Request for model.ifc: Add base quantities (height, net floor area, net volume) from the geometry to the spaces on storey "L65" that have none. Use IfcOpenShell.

First a look at what the model holds.

```python
import ifcopenshell
import ifcopenshell.util.element
import ifcopenshell.util.unit

model = ifcopenshell.open("model.ifc")
print(model.schema)
for unit_type in ("LENGTHUNIT", "AREAUNIT", "VOLUMEUNIT"):
    print(unit_type, ifcopenshell.util.unit.calculate_unit_scale(model, unit_type))
storey = next(s for s in model.by_type("IfcBuildingStorey") if s.Name == "L65")
spaces = [e for e in ifcopenshell.util.element.get_decomposition(storey) if e.is_a("IfcSpace")]
for e in sorted(spaces, key=lambda e: e.id()):
    print(e.id(), e.is_a(), e.Name, list(ifcopenshell.util.element.get_psets(e, qtos_only=True)), sep=" | ")
```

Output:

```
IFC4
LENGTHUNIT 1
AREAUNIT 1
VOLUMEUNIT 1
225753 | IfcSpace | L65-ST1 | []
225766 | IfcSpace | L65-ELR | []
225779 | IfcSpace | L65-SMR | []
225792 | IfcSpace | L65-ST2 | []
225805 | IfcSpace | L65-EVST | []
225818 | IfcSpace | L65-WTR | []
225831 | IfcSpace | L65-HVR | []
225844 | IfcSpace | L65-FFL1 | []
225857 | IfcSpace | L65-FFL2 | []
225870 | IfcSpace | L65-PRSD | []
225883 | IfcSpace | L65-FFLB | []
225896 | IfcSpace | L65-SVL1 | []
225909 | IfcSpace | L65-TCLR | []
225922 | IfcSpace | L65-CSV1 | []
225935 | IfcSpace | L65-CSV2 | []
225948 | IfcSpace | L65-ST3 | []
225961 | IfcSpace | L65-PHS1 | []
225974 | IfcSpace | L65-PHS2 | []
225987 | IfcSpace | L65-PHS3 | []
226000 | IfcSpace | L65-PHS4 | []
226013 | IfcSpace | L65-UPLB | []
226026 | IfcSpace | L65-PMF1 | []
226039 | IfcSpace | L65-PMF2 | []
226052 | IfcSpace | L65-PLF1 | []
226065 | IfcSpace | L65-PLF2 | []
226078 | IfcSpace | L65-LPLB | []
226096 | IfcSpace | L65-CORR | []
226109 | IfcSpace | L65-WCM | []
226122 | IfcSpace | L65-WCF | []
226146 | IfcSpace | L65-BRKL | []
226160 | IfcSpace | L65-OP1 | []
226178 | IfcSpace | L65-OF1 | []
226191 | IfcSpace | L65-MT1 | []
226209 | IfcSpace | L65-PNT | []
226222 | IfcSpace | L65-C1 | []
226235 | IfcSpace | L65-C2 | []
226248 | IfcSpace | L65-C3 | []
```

```python
import ifcopenshell
import ifcopenshell.api.pset
import ifcopenshell.geom
import ifcopenshell.util.element
import ifcopenshell.util.shape
import ifcopenshell.util.unit

model = ifcopenshell.open("model.ifc")
unit_scale = ifcopenshell.util.unit.calculate_unit_scale(model)
area_scale = ifcopenshell.util.unit.calculate_unit_scale(model, "AREAUNIT")
volume_scale = ifcopenshell.util.unit.calculate_unit_scale(model, "VOLUMEUNIT")
settings = ifcopenshell.geom.settings()

storey = next(s for s in model.by_type("IfcBuildingStorey") if s.Name == "L65")
spaces = [e for e in ifcopenshell.util.element.get_decomposition(storey) if e.is_a("IfcSpace")]

for e in sorted(spaces, key=lambda e: e.id()):
    if ifcopenshell.util.element.get_psets(e, qtos_only=True, should_inherit=False):
        continue
    # Geometry comes back in metres, in the element's own axes.
    shape = ifcopenshell.geom.create_shape(settings, e)
    values = {
        "Height": ifcopenshell.util.shape.get_z(shape.geometry) / unit_scale,
        "NetFloorArea": ifcopenshell.util.shape.get_footprint_area(shape.geometry) / area_scale,
        "NetVolume": ifcopenshell.util.shape.get_volume(shape.geometry) / volume_scale,
    }
    qto = ifcopenshell.api.pset.add_qto(model, product=e, name="Qto_SpaceBaseQuantities")
    ifcopenshell.api.pset.edit_qto(model, qto=qto, properties=values)
    print(e.id(), {k: round(v, 3) for k, v in values.items()})

model.write("model_v2.ifc")
```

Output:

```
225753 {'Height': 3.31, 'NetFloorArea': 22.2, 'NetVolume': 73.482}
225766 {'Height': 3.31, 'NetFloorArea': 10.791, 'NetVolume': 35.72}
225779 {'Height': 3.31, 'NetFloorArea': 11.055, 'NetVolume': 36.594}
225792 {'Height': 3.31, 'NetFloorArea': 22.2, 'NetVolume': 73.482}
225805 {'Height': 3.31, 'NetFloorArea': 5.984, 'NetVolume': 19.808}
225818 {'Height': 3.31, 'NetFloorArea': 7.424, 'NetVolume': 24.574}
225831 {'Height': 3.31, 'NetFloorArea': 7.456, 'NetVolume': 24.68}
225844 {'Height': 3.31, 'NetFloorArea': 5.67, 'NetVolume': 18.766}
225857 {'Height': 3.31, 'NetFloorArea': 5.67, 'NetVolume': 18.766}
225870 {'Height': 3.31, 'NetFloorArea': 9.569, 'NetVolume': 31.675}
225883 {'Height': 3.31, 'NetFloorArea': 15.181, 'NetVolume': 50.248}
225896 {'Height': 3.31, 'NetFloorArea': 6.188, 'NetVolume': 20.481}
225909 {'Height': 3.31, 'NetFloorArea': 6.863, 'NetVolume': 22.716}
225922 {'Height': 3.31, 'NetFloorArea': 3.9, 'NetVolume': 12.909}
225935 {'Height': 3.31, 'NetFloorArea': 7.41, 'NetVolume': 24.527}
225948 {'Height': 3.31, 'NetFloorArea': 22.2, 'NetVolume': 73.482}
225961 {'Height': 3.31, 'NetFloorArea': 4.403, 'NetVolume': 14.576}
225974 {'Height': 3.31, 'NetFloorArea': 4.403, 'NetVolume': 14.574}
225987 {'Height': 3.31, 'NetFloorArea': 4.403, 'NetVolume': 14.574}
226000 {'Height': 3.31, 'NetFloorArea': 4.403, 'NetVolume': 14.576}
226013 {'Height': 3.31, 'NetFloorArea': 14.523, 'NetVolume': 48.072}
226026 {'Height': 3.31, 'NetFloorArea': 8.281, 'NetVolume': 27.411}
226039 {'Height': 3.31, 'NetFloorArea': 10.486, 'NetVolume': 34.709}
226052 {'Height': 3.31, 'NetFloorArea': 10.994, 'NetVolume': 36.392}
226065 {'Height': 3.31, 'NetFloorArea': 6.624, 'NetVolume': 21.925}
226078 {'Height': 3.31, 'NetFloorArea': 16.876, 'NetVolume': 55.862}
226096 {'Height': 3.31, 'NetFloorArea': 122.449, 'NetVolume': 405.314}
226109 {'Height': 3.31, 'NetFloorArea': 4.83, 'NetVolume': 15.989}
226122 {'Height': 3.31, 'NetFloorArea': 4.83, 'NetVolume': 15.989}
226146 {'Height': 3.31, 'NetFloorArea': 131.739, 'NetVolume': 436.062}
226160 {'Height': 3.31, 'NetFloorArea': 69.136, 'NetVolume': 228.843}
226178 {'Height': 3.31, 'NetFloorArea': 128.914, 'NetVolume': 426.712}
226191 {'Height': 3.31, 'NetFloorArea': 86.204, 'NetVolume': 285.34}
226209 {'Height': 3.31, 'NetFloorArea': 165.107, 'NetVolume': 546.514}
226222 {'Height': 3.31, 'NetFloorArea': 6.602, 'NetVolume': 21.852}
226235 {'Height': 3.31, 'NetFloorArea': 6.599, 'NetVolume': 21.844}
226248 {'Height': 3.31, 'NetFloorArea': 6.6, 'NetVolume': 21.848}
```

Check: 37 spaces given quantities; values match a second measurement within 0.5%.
